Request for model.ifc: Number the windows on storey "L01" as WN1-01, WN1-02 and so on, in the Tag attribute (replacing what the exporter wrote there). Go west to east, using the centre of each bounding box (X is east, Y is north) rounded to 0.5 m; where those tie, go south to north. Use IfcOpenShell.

First a look at what the model holds.

```python
import ifcopenshell
import ifcopenshell.util.element
import ifcopenshell.util.placement

model = ifcopenshell.open("model.ifc")
print(model.schema)
storey = next(s for s in model.by_type("IfcBuildingStorey") if s.Name == "L01")
windows = [e for e in ifcopenshell.util.element.get_decomposition(storey) if e.is_a("IfcWindow")]
for e in sorted(windows, key=lambda e: e.id()):
    origin = ifcopenshell.util.placement.get_local_placement(e.ObjectPlacement)[:3, 3]
    print(e.id(), e.Tag, e.Name, origin.round(2) + 0.0, sep=" | ")
```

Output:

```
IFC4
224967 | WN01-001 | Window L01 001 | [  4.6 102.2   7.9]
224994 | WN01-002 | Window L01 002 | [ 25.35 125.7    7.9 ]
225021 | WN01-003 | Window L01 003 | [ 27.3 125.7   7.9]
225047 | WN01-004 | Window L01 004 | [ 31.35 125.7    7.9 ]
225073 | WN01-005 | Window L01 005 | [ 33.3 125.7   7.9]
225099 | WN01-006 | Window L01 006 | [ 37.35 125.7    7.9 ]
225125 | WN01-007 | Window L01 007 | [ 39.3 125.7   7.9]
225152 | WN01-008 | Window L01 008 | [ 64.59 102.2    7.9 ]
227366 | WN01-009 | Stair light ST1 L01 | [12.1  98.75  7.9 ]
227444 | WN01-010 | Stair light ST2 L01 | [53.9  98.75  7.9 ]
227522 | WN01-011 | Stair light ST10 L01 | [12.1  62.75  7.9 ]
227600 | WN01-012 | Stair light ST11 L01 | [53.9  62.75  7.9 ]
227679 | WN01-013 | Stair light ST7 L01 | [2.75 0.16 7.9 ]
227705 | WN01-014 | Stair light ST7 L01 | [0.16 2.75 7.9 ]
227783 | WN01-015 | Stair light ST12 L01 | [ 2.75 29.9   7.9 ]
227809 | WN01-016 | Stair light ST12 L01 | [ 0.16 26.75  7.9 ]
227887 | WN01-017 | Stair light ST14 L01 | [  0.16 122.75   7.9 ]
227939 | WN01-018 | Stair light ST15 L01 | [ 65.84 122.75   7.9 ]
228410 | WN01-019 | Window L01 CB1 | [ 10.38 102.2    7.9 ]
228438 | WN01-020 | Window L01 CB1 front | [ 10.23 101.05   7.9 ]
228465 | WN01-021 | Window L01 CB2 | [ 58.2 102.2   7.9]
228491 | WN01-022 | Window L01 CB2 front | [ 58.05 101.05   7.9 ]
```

```python
import ifcopenshell
import ifcopenshell.geom
import ifcopenshell.util.element
import ifcopenshell.util.shape

model = ifcopenshell.open("model.ifc")
settings = ifcopenshell.geom.settings()
settings.set("use-world-coords", True)


def centre(element):
    shape = ifcopenshell.geom.create_shape(settings, element)
    return ifcopenshell.util.shape.get_bbox_centroid(shape.geometry)


storey = next(s for s in model.by_type("IfcBuildingStorey") if s.Name == "L01")
windows = [e for e in ifcopenshell.util.element.get_decomposition(storey) if e.is_a("IfcWindow")]

# Insertion points can sit at a corner or the storey origin, so sort by the geometry (in metres).
centres = {e: centre(e) for e in windows}
windows.sort(key=lambda e: (round(centres[e][0] / 0.5), centres[e][1]))

for i, e in enumerate(windows, start=1):
    number = f"WN1-{i:02d}"
    e.Tag = number
    print(e.id(), number)

model.write("model_v2.ifc")
```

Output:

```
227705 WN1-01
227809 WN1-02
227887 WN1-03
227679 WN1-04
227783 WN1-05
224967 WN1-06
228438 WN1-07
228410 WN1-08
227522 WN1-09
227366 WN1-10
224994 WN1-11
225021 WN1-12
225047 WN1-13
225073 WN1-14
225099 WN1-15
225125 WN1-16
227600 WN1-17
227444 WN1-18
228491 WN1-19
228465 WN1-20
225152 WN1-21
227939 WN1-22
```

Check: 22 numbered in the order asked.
